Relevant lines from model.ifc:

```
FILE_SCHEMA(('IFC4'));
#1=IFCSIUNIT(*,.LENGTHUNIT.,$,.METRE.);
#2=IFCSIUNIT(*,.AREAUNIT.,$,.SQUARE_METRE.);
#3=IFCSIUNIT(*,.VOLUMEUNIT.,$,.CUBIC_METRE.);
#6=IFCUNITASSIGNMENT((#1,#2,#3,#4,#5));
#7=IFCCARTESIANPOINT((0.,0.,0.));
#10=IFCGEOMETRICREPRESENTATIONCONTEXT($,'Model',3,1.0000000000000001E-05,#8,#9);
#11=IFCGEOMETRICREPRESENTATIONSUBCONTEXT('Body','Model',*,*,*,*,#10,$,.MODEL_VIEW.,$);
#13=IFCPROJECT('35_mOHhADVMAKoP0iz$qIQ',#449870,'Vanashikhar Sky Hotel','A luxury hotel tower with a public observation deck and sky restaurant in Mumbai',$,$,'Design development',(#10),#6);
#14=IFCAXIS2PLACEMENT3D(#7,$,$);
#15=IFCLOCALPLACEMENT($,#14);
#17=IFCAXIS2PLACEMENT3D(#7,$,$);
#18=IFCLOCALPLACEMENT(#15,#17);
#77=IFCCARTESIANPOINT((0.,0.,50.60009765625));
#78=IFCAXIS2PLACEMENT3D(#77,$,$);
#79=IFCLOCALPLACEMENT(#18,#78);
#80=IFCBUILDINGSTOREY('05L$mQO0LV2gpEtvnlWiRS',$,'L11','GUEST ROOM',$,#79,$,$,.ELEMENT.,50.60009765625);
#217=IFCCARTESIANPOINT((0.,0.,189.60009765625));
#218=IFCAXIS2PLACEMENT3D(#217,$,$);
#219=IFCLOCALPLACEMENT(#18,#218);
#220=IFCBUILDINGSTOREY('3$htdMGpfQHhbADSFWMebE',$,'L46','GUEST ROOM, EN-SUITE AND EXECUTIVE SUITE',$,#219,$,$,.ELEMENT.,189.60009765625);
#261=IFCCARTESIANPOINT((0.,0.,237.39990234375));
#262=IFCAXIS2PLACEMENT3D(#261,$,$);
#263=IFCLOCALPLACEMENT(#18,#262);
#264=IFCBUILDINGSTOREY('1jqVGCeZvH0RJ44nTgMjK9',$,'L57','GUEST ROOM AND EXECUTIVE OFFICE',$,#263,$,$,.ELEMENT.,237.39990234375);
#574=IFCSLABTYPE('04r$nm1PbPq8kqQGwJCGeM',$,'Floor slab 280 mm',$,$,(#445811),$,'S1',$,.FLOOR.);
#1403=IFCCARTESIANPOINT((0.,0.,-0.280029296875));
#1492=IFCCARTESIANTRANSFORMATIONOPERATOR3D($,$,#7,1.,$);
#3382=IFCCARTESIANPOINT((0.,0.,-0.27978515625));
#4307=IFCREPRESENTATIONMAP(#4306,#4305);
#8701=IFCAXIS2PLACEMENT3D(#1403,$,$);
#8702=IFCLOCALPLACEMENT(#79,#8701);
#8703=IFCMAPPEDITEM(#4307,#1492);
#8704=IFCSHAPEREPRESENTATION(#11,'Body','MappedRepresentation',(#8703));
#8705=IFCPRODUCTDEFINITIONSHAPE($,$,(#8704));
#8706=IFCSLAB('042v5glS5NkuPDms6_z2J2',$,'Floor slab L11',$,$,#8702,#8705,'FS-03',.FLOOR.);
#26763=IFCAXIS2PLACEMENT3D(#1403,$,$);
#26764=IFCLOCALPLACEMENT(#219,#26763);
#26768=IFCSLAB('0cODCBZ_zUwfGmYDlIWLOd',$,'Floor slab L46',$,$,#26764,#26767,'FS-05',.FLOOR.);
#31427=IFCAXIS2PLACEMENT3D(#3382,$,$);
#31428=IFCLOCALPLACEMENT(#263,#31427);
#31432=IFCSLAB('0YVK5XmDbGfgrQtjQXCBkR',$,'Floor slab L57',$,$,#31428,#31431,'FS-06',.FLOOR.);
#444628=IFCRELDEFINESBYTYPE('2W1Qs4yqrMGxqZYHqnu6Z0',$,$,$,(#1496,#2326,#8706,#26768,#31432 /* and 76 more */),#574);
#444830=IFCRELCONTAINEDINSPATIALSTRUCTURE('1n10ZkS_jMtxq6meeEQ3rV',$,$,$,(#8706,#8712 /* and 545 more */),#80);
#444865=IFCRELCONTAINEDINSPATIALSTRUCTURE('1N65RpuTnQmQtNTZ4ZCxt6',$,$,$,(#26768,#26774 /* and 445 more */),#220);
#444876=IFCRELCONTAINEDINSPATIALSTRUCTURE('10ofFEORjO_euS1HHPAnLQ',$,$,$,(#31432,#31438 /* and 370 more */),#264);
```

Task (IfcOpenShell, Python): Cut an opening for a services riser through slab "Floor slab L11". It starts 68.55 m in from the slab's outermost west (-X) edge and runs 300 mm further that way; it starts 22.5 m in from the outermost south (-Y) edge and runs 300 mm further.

```python
import numpy as np
import ifcopenshell
import ifcopenshell.api.feature
import ifcopenshell.api.geometry
import ifcopenshell.api.root
import ifcopenshell.geom
import ifcopenshell.util.placement
import ifcopenshell.util.representation
import ifcopenshell.util.shape
import ifcopenshell.util.unit

model = ifcopenshell.open("model.ifc")
unit_scale = ifcopenshell.util.unit.calculate_unit_scale(model)
settings = ifcopenshell.geom.settings()


def volume(element):
    """Net volume in cubic metres, openings subtracted."""
    shape = ifcopenshell.geom.create_shape(settings, element)
    return ifcopenshell.util.shape.get_volume(shape.geometry)


slab = model.by_id(8706)
before = volume(slab)

# Extent in the slab's own axes, in metres. The edges named are its -X and -Y sides.
slab_shape = ifcopenshell.geom.create_shape(settings, slab)
vertices = ifcopenshell.util.shape.get_vertices(slab_shape.geometry)
x_min, y_min, bottom = vertices.min(axis=0)
top = vertices[:, 2].max()

opening = ifcopenshell.api.root.create_entity(model, ifc_class="IfcOpeningElement", name="Services riser opening", predefined_type="OPENING")
context = ifcopenshell.util.representation.get_context(model, "Model", "Body", "MODEL_VIEW")
width, depth = 0.3, 0.3
outline = [(0.0, 0.0), (width, 0.0), (width, depth), (0.0, depth), (0.0, 0.0)]
# Overshoot both faces by 50 mm so the cut is clean.
shape = ifcopenshell.api.geometry.add_slab_representation(
    model, context=context, depth=top - bottom + 0.1, polyline=outline
)
ifcopenshell.api.geometry.assign_representation(model, product=opening, representation=shape)

matrix = ifcopenshell.util.placement.get_local_placement(slab.ObjectPlacement)
matrix[:, 3] = matrix @ np.append(np.array([x_min + 68.55, y_min + 22.5, bottom - 0.05]) / unit_scale, 1.0)
ifcopenshell.api.geometry.edit_object_placement(model, product=opening, matrix=matrix, is_si=False)
ifcopenshell.api.feature.add_feature(model, feature=opening, element=slab)

after = volume(slab)

print(f"slab volume {before:.3f} -> {after:.3f} m3")

model.write("model_edited.ifc")
```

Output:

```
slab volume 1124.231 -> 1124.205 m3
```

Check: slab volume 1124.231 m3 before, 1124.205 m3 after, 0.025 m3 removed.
